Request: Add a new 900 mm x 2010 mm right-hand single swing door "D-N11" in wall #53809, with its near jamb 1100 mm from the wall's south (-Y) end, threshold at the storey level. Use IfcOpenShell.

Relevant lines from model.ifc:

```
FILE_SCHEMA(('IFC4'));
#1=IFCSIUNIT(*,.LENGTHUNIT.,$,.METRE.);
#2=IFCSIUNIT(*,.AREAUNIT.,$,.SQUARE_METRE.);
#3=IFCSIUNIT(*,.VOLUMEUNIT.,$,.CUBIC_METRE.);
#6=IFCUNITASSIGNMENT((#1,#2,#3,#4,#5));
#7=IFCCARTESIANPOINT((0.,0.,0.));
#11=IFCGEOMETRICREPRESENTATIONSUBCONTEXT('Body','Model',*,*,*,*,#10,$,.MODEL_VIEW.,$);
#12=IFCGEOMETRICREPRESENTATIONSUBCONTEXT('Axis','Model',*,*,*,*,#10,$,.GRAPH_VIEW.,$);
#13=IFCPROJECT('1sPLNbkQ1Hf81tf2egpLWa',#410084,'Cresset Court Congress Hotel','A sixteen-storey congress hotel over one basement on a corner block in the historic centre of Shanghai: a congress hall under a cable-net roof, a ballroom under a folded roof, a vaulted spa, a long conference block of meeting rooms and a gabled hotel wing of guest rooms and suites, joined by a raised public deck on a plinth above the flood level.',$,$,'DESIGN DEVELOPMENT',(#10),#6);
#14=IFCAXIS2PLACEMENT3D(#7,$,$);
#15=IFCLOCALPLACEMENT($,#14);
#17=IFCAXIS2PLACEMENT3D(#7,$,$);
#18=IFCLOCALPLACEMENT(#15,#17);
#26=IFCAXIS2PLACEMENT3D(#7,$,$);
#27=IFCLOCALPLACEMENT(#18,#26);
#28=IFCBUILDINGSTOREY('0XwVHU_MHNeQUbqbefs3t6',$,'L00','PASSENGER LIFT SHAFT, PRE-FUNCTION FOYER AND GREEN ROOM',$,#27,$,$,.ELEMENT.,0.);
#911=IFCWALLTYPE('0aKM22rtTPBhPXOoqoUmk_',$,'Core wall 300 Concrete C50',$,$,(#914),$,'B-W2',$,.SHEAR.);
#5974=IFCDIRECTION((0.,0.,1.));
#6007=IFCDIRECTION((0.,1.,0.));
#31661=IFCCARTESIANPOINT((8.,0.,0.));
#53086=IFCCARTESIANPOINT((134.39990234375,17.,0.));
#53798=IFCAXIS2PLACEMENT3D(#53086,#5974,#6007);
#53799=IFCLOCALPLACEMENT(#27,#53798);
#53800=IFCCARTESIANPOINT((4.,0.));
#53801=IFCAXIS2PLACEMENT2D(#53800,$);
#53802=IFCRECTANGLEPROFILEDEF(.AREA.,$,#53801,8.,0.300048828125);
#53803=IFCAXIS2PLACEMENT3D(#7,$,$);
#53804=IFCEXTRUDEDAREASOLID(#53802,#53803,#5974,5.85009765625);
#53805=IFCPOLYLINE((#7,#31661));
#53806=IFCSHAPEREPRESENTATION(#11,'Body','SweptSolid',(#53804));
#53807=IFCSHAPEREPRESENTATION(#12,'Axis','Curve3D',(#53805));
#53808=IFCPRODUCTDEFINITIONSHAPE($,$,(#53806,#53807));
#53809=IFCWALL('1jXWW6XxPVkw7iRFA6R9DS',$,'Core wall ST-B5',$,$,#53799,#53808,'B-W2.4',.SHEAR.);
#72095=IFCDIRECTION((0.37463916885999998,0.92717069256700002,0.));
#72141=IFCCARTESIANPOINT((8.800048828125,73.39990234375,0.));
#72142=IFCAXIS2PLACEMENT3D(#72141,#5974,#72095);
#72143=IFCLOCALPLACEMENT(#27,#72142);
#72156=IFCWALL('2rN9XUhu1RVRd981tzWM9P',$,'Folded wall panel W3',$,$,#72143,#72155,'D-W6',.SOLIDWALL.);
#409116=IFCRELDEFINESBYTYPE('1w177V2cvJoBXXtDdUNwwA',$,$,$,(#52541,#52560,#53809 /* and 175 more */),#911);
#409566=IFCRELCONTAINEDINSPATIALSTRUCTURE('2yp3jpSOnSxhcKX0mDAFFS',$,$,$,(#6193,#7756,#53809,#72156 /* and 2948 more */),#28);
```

```python
import numpy as np
import ifcopenshell
import ifcopenshell.api.feature
import ifcopenshell.api.geometry
import ifcopenshell.api.root
import ifcopenshell.api.spatial
import ifcopenshell.geom
import ifcopenshell.util.element
import ifcopenshell.util.placement
import ifcopenshell.util.representation
import ifcopenshell.util.shape
import ifcopenshell.util.unit

model = ifcopenshell.open("model.ifc")
unit_scale = ifcopenshell.util.unit.calculate_unit_scale(model)
settings = ifcopenshell.geom.settings()


def volume(element):
    """Net volume in cubic metres, openings subtracted."""
    shape = ifcopenshell.geom.create_shape(settings, element)
    return ifcopenshell.util.shape.get_volume(shape.geometry)


wall = model.by_id(53809)
storey = ifcopenshell.util.element.get_container(wall, ifc_class="IfcBuildingStorey")
context = ifcopenshell.util.representation.get_context(model, "Model", "Body", "MODEL_VIEW")
before = volume(wall)

width, height, from_end, sill = 0.9, 2.01, 1.1, 0.0  # metres

# The wall runs along its own X axis, and the end named is its -X end.
wall_shape = ifcopenshell.geom.create_shape(settings, wall)
x, y, z = ifcopenshell.util.shape.get_vertices(wall_shape.geometry).T
start = x.min() + from_end
face, thickness = float(y.min()), float(y.max() - y.min())
wall_matrix = ifcopenshell.util.placement.get_local_placement(wall.ObjectPlacement)
level = ifcopenshell.util.placement.get_local_placement(storey.ObjectPlacement)[2, 3]


def in_wall(x, y):
    """Placement at x, y metres in the wall's axes, at sill height."""
    matrix = wall_matrix.copy()
    matrix[:, 3] = wall_matrix @ np.array([x / unit_scale, y / unit_scale, 0.0, 1.0])
    matrix[2, 3] = level + sill / unit_scale
    return matrix


# Opening: a box that overshoots both wall faces by 50 mm.
opening = ifcopenshell.api.root.create_entity(model, ifc_class="IfcOpeningElement", predefined_type="OPENING")
box = ifcopenshell.api.geometry.add_wall_representation(
    model, context=context, length=width, height=height, thickness=thickness + 0.1
)
ifcopenshell.api.geometry.assign_representation(model, product=opening, representation=box)
ifcopenshell.api.geometry.edit_object_placement(model, product=opening, matrix=in_wall(start, face - 0.05), is_si=False)
ifcopenshell.api.feature.add_feature(model, feature=opening, element=wall)

door = ifcopenshell.api.root.create_entity(model, ifc_class="IfcDoor", name="D-N11", predefined_type="DOOR")
door.OverallWidth, door.OverallHeight = width / unit_scale, height / unit_scale
door.OperationType = "SINGLE_SWING_RIGHT"
body = ifcopenshell.api.geometry.add_door_representation(
    model,
    context=context,
    overall_width=door.OverallWidth,
    overall_height=door.OverallHeight,
    operation_type="SINGLE_SWING_RIGHT",
    lining_properties={"LiningDepth": thickness / unit_scale, "ThresholdDepth": thickness / unit_scale},
)
ifcopenshell.api.geometry.assign_representation(model, product=door, representation=body)
ifcopenshell.api.spatial.assign_container(model, products=[door], relating_structure=storey)
ifcopenshell.api.feature.add_filling(model, opening=opening, element=door)

# The lining spans the wall, so the door starts at the wall face.
ifcopenshell.api.geometry.edit_object_placement(model, product=door, matrix=in_wall(start, face), is_si=False)

after = volume(wall)

print(f"wall volume {before:.3f} -> {after:.3f} m3")

model.write("model-out.ifc")
```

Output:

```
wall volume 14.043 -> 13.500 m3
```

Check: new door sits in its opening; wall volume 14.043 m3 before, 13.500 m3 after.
